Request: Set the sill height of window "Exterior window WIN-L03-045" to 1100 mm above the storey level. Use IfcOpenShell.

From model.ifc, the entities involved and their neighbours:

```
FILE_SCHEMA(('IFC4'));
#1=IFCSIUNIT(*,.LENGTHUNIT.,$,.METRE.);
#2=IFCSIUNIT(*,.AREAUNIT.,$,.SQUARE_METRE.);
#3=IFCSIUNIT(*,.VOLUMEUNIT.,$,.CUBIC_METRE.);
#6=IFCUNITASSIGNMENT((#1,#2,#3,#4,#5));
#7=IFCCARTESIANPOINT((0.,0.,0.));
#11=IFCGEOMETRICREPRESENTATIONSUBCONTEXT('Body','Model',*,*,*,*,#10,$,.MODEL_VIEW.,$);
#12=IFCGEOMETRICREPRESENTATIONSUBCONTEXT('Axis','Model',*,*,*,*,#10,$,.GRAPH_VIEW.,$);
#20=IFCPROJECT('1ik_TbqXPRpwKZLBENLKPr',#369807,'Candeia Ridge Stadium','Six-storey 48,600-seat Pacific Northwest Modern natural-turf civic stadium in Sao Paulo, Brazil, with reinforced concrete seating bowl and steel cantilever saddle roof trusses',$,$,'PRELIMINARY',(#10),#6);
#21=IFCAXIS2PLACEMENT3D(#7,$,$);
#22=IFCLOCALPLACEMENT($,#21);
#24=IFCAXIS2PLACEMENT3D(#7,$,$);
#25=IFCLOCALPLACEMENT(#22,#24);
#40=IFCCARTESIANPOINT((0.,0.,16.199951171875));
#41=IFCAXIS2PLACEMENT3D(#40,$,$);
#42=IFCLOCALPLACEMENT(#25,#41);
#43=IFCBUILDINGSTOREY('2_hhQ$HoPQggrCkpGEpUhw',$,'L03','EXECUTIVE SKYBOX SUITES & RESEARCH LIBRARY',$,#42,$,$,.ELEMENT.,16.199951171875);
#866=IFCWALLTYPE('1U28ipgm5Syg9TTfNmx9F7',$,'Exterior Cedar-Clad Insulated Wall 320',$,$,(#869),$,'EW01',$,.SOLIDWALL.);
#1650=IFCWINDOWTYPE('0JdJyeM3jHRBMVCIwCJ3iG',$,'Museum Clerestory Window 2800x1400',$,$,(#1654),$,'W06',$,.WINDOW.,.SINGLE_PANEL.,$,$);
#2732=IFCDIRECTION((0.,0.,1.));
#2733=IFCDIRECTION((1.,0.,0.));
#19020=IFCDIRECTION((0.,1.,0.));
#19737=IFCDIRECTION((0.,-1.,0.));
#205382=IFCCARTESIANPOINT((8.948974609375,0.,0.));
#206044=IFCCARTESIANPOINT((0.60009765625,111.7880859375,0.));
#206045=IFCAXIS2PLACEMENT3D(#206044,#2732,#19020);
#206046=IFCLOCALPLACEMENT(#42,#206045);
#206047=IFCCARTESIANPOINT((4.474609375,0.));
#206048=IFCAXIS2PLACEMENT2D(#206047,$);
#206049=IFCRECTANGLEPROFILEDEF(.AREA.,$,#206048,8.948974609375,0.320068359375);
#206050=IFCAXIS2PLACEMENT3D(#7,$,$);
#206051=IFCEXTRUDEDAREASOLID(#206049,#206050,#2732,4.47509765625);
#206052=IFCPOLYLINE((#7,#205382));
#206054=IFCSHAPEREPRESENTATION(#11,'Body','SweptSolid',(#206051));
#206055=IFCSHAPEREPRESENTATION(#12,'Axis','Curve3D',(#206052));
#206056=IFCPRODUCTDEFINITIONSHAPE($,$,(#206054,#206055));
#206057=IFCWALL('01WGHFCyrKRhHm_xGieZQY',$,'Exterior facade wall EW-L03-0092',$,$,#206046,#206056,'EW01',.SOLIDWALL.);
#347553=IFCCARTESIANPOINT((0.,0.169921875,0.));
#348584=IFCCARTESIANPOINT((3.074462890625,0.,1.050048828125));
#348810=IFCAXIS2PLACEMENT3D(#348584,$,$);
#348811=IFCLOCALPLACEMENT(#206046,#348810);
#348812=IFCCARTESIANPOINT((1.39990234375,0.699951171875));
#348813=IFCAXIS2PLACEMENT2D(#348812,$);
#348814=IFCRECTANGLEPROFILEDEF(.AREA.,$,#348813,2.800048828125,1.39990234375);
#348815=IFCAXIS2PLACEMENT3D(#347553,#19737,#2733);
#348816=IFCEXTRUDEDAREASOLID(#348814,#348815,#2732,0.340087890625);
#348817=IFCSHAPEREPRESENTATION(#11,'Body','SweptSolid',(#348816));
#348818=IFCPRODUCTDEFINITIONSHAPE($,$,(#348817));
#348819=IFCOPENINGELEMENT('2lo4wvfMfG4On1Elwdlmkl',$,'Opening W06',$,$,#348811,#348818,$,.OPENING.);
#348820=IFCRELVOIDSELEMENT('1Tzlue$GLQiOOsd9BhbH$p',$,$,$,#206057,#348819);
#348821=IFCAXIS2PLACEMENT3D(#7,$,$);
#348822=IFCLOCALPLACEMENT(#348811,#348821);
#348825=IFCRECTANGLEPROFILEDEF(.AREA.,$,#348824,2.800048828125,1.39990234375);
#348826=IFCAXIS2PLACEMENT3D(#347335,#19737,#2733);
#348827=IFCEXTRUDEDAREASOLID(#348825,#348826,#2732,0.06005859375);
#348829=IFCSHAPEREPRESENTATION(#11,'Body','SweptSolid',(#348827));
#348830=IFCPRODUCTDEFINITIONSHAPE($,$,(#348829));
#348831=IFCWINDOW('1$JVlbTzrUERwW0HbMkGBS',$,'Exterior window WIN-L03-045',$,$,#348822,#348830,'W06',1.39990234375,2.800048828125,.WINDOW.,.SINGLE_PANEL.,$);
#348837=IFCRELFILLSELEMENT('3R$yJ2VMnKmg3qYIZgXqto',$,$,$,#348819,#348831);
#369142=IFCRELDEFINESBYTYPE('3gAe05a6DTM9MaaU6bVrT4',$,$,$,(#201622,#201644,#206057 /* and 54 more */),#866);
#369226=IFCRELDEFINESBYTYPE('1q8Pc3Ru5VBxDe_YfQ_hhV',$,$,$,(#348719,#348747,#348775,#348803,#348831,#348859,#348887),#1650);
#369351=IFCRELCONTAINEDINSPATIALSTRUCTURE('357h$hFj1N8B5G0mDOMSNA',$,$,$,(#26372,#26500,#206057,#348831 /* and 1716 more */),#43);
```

```python
import numpy as np
import ifcopenshell
import ifcopenshell.api.geometry
import ifcopenshell.geom
import ifcopenshell.util.element
import ifcopenshell.util.placement
import ifcopenshell.util.shape
import ifcopenshell.util.unit

model = ifcopenshell.open("model.ifc")
unit_scale = ifcopenshell.util.unit.calculate_unit_scale(model)

window = model.by_id(348831)
opening = window.FillsVoids[0].RelatingOpeningElement
storey = ifcopenshell.util.element.get_container(window, ifc_class="IfcBuildingStorey")
level = ifcopenshell.util.placement.get_local_placement(storey.ObjectPlacement)[2, 3]

# The opening's origin need not be at the sill, so measure its lowest point.
shape = ifcopenshell.geom.create_shape(ifcopenshell.geom.settings(), opening)
bottom = ifcopenshell.util.shape.get_shape_bottom_elevation(shape, shape.geometry) / unit_scale
dz = level + 1.1 - bottom

shift = np.array([0.0, 0.0, dz])
# The window is placed relative to its opening, so it follows when the opening moves.
matrix = ifcopenshell.util.placement.get_local_placement(opening.ObjectPlacement)
matrix[:3, 3] += shift
ifcopenshell.api.geometry.edit_object_placement(
    model, product=opening, matrix=matrix, is_si=False, should_transform_children=True
)

print(f"moved by {dz * unit_scale:+.3f} m")

model.write("model_rev.ifc")
```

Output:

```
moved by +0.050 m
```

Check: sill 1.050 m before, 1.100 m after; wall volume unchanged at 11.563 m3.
